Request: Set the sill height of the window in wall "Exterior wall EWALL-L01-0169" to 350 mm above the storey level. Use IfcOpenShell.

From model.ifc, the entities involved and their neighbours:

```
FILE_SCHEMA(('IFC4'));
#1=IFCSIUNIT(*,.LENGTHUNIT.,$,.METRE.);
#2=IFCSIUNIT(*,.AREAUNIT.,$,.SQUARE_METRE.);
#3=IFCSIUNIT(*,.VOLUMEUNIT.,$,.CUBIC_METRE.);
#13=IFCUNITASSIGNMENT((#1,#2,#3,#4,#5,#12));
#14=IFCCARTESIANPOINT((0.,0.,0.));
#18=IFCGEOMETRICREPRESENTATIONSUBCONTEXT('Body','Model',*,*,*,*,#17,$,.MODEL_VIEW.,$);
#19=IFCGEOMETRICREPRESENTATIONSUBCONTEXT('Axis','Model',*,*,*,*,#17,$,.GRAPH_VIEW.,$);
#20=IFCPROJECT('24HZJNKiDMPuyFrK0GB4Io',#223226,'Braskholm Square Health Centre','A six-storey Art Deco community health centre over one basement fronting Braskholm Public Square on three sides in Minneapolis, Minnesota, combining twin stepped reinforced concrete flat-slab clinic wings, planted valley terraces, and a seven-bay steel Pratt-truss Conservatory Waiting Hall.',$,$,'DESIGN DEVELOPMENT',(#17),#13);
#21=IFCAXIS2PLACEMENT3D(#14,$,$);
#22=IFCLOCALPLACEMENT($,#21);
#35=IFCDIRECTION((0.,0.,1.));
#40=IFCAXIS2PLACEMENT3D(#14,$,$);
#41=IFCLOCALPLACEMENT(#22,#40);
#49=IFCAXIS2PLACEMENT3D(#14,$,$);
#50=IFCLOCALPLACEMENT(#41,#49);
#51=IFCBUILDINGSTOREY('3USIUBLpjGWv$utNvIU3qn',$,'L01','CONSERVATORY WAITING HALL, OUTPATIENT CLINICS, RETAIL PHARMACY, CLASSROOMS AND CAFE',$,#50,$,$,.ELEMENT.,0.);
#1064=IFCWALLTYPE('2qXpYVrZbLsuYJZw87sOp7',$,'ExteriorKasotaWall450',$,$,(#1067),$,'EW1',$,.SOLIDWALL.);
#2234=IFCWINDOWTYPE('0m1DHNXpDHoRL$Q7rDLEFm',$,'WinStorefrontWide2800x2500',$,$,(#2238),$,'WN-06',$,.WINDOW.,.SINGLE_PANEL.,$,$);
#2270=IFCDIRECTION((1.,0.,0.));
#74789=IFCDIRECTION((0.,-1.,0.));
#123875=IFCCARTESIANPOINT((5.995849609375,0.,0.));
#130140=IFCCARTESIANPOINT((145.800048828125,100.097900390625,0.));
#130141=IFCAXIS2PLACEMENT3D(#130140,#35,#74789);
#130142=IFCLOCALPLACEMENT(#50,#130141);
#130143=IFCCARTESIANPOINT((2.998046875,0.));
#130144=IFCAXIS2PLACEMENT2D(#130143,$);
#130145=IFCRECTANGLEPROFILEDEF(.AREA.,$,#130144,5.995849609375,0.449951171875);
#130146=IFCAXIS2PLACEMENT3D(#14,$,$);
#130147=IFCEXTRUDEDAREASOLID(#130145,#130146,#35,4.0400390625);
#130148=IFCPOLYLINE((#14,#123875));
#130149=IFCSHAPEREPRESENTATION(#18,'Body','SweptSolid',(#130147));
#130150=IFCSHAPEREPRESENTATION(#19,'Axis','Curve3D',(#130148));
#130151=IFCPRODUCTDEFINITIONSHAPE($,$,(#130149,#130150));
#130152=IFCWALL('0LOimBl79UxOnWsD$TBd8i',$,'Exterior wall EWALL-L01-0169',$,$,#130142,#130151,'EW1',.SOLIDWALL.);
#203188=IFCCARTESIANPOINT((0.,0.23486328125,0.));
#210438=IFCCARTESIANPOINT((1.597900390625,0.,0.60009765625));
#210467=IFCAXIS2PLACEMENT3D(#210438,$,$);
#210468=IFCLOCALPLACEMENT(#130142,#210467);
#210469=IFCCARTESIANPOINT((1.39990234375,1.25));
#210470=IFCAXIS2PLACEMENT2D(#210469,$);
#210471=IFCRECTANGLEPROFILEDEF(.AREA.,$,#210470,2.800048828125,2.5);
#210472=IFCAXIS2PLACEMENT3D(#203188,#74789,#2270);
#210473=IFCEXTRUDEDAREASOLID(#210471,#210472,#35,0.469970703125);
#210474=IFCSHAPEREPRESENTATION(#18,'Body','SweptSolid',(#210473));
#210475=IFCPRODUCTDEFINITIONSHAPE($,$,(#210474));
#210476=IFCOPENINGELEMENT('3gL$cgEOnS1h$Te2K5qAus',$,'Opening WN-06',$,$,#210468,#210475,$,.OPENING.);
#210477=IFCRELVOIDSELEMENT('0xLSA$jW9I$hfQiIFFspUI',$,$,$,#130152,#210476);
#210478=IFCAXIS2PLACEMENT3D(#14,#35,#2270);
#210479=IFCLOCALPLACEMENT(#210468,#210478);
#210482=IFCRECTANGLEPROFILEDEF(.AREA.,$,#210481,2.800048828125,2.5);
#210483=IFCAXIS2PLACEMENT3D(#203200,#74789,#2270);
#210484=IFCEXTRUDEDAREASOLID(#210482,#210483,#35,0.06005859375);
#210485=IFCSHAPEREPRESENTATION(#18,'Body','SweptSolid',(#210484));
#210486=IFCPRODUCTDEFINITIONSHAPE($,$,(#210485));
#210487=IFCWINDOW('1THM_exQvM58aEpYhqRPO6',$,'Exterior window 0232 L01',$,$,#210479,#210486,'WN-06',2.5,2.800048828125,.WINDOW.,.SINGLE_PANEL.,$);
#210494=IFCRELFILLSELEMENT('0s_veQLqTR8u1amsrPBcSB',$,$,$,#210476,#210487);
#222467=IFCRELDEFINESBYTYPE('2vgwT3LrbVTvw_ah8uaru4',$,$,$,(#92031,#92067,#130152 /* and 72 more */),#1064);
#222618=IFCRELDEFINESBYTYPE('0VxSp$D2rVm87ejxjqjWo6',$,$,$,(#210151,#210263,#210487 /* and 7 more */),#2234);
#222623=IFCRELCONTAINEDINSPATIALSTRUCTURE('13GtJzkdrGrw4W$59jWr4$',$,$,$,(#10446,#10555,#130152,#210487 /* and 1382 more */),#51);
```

```python
import numpy as np
import ifcopenshell
import ifcopenshell.api.geometry
import ifcopenshell.geom
import ifcopenshell.util.element
import ifcopenshell.util.placement
import ifcopenshell.util.shape
import ifcopenshell.util.unit

model = ifcopenshell.open("model.ifc")
unit_scale = ifcopenshell.util.unit.calculate_unit_scale(model)

window = model.by_guid("1THM_exQvM58aEpYhqRPO6")
opening = window.FillsVoids[0].RelatingOpeningElement
storey = ifcopenshell.util.element.get_container(window, ifc_class="IfcBuildingStorey")
level = ifcopenshell.util.placement.get_local_placement(storey.ObjectPlacement)[2, 3]

# The opening's origin need not be at the sill, so measure its lowest point.
shape = ifcopenshell.geom.create_shape(ifcopenshell.geom.settings(), opening)
bottom = ifcopenshell.util.shape.get_shape_bottom_elevation(shape, shape.geometry) / unit_scale
dz = level + 0.35 - bottom

shift = np.array([0.0, 0.0, dz])
# The window is placed relative to its opening, so it follows when the opening moves.
matrix = ifcopenshell.util.placement.get_local_placement(opening.ObjectPlacement)
matrix[:3, 3] += shift
ifcopenshell.api.geometry.edit_object_placement(
    model, product=opening, matrix=matrix, is_si=False, should_transform_children=True
)

print(f"moved by {dz * unit_scale:+.3f} m")

model.write("model_v2.ifc")
```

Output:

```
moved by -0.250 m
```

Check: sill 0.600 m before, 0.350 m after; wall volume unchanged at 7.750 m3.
